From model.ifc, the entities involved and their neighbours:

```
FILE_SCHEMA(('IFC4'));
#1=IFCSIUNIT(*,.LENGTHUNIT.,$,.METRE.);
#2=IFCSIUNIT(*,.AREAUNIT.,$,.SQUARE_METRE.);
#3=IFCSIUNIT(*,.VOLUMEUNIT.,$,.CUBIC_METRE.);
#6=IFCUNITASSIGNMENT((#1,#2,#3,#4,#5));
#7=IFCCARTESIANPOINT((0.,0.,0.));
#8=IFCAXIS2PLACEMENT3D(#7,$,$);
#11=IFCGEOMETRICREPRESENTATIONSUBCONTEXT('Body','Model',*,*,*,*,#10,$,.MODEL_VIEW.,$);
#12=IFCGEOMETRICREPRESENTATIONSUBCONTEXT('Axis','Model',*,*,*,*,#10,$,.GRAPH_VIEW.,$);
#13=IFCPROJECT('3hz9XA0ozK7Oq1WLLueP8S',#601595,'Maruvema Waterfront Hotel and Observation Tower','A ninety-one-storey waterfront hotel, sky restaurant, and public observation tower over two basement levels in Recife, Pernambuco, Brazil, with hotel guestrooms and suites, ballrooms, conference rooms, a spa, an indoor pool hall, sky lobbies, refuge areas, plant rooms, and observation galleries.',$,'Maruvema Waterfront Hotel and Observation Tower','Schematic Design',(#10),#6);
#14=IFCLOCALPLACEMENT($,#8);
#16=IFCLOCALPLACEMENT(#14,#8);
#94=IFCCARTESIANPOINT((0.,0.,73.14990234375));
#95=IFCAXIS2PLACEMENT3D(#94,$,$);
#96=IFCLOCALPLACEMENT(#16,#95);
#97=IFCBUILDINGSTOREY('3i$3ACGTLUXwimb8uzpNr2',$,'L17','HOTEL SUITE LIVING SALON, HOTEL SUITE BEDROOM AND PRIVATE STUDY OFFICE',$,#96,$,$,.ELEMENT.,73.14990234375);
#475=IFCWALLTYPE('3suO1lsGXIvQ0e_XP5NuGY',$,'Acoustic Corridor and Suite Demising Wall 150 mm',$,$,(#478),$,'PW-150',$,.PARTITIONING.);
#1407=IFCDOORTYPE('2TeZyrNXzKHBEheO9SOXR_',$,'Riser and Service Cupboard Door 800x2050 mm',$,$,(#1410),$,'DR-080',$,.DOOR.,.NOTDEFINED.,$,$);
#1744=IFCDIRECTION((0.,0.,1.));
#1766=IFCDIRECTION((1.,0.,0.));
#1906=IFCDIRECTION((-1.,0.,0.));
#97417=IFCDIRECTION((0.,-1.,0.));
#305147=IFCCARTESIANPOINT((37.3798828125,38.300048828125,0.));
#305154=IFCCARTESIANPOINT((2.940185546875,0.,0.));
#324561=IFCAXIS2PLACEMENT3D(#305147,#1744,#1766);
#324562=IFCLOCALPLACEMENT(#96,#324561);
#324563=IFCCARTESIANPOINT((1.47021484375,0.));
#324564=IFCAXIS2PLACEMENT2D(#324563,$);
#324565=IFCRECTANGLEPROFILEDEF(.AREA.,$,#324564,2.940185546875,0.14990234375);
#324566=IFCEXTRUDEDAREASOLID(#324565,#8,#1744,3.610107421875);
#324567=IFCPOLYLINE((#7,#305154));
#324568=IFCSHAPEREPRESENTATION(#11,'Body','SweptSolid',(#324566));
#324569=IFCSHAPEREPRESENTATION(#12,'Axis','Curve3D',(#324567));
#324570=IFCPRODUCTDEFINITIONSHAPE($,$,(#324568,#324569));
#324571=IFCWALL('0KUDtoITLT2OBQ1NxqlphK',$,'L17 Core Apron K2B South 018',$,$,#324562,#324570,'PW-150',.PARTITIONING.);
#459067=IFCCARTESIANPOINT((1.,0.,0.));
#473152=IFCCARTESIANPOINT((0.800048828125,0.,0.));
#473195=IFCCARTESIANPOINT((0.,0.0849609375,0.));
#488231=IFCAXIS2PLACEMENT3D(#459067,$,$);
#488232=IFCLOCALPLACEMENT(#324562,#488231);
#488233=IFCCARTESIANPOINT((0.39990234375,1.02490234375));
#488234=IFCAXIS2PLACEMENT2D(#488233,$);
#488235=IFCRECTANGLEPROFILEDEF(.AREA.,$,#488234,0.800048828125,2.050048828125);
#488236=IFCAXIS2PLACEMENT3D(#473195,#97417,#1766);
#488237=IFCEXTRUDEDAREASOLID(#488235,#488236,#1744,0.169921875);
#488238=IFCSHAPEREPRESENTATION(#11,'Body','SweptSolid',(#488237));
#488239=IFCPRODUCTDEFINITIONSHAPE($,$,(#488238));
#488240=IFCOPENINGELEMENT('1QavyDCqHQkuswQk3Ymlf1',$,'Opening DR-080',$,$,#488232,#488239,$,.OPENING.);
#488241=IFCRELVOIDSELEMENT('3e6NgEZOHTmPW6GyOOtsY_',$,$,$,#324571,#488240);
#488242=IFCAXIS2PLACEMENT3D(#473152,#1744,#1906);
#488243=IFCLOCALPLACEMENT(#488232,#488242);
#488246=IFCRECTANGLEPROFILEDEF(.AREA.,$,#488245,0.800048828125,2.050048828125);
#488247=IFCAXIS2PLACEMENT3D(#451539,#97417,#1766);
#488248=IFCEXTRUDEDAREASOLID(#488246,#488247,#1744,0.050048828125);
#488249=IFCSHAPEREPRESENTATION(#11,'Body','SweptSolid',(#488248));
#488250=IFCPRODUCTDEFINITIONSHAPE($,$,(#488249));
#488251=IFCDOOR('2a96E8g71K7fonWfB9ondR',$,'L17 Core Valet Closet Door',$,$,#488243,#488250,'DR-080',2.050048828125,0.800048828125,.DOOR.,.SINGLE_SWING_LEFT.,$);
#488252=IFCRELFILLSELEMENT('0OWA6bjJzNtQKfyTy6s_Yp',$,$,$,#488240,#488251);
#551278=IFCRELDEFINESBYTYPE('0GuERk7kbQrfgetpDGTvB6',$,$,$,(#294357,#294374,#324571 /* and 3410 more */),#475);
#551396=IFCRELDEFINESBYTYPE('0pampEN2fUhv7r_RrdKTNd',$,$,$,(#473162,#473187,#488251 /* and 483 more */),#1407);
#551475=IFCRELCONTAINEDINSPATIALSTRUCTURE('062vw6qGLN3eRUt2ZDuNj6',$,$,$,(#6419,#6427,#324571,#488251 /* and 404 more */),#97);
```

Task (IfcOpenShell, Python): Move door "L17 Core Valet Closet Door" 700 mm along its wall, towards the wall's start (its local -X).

```python
import ifcopenshell
import ifcopenshell.api.geometry
import ifcopenshell.util.placement
import ifcopenshell.util.unit

model = ifcopenshell.open("model.ifc")
unit_scale = ifcopenshell.util.unit.calculate_unit_scale(model)

door = model.by_id(488251)
opening = door.FillsVoids[0].RelatingOpeningElement
wall = opening.VoidsElements[0].RelatingBuildingElement

wall_matrix = ifcopenshell.util.placement.get_local_placement(wall.ObjectPlacement)
shift = wall_matrix[:3, 0] * -0.7 / unit_scale
before = ifcopenshell.util.placement.get_local_placement(door.ObjectPlacement)[:3, 3].copy()

# The door is placed relative to its opening, so it follows when the opening moves.
matrix = ifcopenshell.util.placement.get_local_placement(opening.ObjectPlacement)
matrix[:3, 3] += shift
ifcopenshell.api.geometry.edit_object_placement(
    model, product=opening, matrix=matrix, is_si=False, should_transform_children=True
)

after = ifcopenshell.util.placement.get_local_placement(door.ObjectPlacement)[:3, 3]
print("door moved by", (after - before).round(3) + 0.0)

model.write("model_updated.ifc")
```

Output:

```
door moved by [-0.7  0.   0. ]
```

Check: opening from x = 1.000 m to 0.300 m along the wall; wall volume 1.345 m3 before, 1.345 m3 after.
